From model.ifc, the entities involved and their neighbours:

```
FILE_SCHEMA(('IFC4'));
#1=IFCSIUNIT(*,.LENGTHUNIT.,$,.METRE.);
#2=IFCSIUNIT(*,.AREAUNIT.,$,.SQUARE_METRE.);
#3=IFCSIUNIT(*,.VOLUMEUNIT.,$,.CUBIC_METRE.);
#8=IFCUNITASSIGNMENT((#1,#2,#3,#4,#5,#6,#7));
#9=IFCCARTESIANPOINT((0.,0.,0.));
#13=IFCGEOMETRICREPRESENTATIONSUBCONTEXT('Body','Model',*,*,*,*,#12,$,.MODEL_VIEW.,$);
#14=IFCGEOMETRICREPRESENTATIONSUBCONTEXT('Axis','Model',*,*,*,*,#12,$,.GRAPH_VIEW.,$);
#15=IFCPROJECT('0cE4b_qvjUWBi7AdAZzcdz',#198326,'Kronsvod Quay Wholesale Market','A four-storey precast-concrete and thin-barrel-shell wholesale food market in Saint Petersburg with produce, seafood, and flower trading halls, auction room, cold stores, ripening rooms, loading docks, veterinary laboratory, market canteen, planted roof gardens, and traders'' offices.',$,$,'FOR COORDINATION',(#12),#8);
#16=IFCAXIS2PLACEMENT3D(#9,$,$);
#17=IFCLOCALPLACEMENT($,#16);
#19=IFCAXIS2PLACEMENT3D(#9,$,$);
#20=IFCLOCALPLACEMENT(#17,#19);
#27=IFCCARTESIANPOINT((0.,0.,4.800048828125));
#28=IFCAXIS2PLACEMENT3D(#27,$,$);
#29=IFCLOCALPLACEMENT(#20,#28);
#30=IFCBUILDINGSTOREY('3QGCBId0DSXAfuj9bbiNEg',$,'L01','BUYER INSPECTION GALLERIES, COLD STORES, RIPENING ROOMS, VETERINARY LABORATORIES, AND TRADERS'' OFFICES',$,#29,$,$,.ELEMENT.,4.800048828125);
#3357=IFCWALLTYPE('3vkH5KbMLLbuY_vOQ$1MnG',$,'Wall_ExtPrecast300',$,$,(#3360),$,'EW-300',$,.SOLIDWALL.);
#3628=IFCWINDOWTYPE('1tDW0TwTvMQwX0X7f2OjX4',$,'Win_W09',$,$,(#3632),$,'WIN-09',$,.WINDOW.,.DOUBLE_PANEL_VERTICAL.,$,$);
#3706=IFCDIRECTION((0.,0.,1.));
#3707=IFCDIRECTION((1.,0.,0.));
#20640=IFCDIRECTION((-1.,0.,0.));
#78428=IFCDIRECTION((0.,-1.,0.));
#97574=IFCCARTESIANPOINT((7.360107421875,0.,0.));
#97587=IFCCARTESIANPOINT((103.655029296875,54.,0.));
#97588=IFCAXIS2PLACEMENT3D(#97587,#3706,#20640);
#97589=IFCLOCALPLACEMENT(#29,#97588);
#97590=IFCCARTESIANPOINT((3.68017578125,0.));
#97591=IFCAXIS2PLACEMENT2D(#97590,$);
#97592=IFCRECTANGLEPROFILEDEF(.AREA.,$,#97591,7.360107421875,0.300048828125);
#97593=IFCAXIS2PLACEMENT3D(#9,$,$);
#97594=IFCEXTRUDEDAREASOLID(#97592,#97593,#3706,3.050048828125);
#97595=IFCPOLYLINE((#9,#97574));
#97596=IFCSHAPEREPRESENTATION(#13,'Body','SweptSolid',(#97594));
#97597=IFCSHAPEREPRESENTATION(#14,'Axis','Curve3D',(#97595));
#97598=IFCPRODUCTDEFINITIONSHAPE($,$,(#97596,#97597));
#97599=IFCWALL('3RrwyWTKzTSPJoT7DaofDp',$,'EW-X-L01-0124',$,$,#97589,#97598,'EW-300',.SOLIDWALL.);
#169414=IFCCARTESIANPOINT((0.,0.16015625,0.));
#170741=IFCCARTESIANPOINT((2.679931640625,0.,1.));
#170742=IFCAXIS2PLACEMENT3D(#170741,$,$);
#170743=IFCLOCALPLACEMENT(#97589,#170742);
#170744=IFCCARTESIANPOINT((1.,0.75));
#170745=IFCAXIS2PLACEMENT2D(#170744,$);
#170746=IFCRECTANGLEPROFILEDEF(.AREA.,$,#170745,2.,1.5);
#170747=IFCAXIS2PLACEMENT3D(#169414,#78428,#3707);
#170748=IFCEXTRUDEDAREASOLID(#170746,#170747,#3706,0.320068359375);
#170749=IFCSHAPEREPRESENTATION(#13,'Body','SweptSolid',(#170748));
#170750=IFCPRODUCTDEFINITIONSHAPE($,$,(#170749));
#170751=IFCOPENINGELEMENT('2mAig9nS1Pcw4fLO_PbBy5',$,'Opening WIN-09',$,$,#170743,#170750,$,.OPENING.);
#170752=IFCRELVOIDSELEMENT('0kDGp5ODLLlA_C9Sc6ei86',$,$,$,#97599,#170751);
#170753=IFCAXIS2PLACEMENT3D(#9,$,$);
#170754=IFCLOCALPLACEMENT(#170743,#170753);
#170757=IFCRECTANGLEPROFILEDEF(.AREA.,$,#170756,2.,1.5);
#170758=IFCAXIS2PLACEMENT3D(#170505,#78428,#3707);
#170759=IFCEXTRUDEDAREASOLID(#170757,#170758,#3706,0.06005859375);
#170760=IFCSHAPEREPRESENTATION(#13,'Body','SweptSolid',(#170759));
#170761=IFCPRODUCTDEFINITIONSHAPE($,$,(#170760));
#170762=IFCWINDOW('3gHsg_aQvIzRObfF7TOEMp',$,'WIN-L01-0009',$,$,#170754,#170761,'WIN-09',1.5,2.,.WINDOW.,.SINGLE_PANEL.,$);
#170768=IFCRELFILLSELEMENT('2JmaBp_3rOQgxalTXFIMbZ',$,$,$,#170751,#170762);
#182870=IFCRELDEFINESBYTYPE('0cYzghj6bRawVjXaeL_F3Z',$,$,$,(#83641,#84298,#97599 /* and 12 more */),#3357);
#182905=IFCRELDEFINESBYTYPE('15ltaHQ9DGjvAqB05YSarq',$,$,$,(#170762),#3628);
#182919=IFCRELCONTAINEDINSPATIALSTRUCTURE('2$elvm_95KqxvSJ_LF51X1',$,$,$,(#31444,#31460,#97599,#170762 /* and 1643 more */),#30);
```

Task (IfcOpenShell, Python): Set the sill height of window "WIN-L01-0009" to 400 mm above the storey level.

```python
import numpy as np
import ifcopenshell
import ifcopenshell.api.geometry
import ifcopenshell.geom
import ifcopenshell.util.element
import ifcopenshell.util.placement
import ifcopenshell.util.shape
import ifcopenshell.util.unit

model = ifcopenshell.open("model.ifc")
unit_scale = ifcopenshell.util.unit.calculate_unit_scale(model)

window = model.by_guid("3gHsg_aQvIzRObfF7TOEMp")
opening = window.FillsVoids[0].RelatingOpeningElement
storey = ifcopenshell.util.element.get_container(window, ifc_class="IfcBuildingStorey")
level = ifcopenshell.util.placement.get_local_placement(storey.ObjectPlacement)[2, 3]

# The opening's origin need not be at the sill, so measure its lowest point.
shape = ifcopenshell.geom.create_shape(ifcopenshell.geom.settings(), opening)
bottom = ifcopenshell.util.shape.get_shape_bottom_elevation(shape, shape.geometry) / unit_scale
dz = level + 0.4 - bottom

shift = np.array([0.0, 0.0, dz])
# The window is placed relative to its opening, so it follows when the opening moves.
matrix = ifcopenshell.util.placement.get_local_placement(opening.ObjectPlacement)
matrix[:3, 3] += shift
ifcopenshell.api.geometry.edit_object_placement(
    model, product=opening, matrix=matrix, is_si=False, should_transform_children=True
)

print(f"moved by {dz * unit_scale:+.3f} m")

model.write("model_edited.ifc")
```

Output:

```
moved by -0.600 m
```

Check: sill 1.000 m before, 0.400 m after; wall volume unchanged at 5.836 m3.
